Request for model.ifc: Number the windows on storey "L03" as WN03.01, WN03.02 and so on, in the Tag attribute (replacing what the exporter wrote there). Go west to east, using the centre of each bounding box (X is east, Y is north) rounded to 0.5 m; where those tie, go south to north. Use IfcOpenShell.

First a look at what the model holds.

```python
import ifcopenshell
import ifcopenshell.util.element
import ifcopenshell.util.placement

model = ifcopenshell.open("model.ifc")
print(model.schema)
storey = next(s for s in model.by_type("IfcBuildingStorey") if s.Name == "L03")
windows = [e for e in ifcopenshell.util.element.get_decomposition(storey) if e.is_a("IfcWindow")]
for e in sorted(windows, key=lambda e: e.id()):
    origin = ifcopenshell.util.placement.get_local_placement(e.ObjectPlacement)[:3, 3]
    print(e.id(), e.Tag, e.Name, origin.round(2) + 0.0, sep=" | ")
```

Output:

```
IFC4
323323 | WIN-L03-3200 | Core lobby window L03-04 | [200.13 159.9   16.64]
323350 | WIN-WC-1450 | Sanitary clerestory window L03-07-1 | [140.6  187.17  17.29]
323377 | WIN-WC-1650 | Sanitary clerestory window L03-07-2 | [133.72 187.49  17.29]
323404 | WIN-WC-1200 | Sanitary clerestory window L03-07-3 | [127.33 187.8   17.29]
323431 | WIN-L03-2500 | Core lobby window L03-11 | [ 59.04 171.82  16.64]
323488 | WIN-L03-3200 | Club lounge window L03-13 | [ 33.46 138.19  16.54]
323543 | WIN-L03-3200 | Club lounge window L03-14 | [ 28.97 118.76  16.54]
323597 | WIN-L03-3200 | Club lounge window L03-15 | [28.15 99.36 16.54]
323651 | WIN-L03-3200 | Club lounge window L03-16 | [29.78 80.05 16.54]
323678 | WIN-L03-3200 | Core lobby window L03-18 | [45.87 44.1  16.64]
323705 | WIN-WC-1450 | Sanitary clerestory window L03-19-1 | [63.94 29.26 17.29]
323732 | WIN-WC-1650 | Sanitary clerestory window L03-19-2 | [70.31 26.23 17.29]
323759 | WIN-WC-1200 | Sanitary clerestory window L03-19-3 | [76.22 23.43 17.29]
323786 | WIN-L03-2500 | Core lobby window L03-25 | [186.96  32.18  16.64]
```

```python
import ifcopenshell
import ifcopenshell.geom
import ifcopenshell.util.element
import ifcopenshell.util.shape

model = ifcopenshell.open("model.ifc")
settings = ifcopenshell.geom.settings()
settings.set("use-world-coords", True)


def centre(element):
    shape = ifcopenshell.geom.create_shape(settings, element)
    return ifcopenshell.util.shape.get_bbox_centroid(shape.geometry)


storey = next(s for s in model.by_type("IfcBuildingStorey") if s.Name == "L03")
windows = [e for e in ifcopenshell.util.element.get_decomposition(storey) if e.is_a("IfcWindow")]

# Insertion points can sit at a corner or the storey origin, so sort by the geometry (in metres).
centres = {e: centre(e) for e in windows}
windows.sort(key=lambda e: (round(centres[e][0] / 0.5), centres[e][1]))

for i, e in enumerate(windows, start=1):
    number = f"WN03.{i:02d}"
    e.Tag = number
    print(e.id(), number)

model.write("model_v2.ifc")
```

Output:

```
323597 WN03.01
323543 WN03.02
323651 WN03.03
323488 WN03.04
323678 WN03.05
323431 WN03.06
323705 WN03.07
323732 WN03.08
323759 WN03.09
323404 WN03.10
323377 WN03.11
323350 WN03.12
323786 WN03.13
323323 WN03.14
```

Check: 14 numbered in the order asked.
